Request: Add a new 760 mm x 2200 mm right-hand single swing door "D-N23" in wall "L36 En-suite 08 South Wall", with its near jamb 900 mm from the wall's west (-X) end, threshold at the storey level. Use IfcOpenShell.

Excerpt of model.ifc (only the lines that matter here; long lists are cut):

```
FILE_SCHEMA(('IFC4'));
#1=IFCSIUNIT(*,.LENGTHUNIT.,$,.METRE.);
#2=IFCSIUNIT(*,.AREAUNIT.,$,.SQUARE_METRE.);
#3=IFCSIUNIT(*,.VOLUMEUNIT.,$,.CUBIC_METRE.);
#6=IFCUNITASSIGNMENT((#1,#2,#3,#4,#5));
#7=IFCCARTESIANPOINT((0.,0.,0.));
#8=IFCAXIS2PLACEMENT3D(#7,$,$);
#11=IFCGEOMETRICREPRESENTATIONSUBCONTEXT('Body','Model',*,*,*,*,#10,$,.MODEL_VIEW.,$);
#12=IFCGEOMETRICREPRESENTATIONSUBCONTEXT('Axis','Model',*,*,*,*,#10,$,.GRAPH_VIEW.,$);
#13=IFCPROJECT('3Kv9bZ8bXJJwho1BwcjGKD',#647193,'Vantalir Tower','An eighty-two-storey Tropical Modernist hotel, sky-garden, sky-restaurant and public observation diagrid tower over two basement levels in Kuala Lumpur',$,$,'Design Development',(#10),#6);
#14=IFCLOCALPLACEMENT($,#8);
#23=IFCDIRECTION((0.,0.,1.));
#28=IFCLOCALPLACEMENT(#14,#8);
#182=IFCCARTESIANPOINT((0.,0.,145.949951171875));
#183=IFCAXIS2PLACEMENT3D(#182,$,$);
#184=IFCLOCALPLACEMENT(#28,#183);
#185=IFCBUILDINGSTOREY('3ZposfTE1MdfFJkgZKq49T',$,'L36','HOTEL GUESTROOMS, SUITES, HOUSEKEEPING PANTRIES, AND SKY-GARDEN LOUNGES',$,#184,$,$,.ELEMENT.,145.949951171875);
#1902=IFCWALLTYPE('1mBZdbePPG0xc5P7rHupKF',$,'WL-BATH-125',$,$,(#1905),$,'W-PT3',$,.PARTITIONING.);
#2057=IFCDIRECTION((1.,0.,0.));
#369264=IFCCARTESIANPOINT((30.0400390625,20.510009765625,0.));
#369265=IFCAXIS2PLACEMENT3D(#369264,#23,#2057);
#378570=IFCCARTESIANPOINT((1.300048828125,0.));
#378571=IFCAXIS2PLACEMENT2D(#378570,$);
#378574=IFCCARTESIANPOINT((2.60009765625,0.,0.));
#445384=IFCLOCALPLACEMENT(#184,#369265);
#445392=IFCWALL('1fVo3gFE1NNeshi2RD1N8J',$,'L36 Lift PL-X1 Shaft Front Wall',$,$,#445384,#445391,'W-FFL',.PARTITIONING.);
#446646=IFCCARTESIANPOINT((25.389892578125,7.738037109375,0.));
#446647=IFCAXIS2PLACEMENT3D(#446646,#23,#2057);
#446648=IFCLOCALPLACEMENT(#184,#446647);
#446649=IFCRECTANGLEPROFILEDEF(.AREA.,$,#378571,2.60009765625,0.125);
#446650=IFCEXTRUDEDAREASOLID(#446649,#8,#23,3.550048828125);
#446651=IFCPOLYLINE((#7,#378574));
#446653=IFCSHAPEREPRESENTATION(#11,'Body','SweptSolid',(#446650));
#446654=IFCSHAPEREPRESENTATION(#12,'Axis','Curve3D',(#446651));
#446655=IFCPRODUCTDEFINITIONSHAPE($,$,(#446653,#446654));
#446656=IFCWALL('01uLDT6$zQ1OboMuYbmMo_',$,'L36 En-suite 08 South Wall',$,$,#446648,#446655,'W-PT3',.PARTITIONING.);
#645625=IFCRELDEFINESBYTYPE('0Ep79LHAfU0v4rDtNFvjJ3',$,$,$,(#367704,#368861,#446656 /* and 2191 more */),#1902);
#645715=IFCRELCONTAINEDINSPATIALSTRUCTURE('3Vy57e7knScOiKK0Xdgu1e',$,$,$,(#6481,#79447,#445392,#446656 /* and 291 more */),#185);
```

```python
import numpy as np
import ifcopenshell
import ifcopenshell.api.feature
import ifcopenshell.api.geometry
import ifcopenshell.api.root
import ifcopenshell.api.spatial
import ifcopenshell.geom
import ifcopenshell.util.element
import ifcopenshell.util.placement
import ifcopenshell.util.representation
import ifcopenshell.util.shape
import ifcopenshell.util.unit

model = ifcopenshell.open("model.ifc")
unit_scale = ifcopenshell.util.unit.calculate_unit_scale(model)
settings = ifcopenshell.geom.settings()


def volume(element):
    """Net volume in cubic metres, openings subtracted."""
    shape = ifcopenshell.geom.create_shape(settings, element)
    return ifcopenshell.util.shape.get_volume(shape.geometry)


wall = model.by_guid("01uLDT6$zQ1OboMuYbmMo_")
storey = ifcopenshell.util.element.get_container(wall, ifc_class="IfcBuildingStorey")
context = ifcopenshell.util.representation.get_context(model, "Model", "Body", "MODEL_VIEW")
before = volume(wall)

width, height, from_end, sill = 0.76, 2.2, 0.9, 0.0  # metres

# The wall runs along its own X axis, and the end named is its -X end.
wall_shape = ifcopenshell.geom.create_shape(settings, wall)
x, y, z = ifcopenshell.util.shape.get_vertices(wall_shape.geometry).T
start = x.min() + from_end
face, thickness = float(y.min()), float(y.max() - y.min())
wall_matrix = ifcopenshell.util.placement.get_local_placement(wall.ObjectPlacement)
level = ifcopenshell.util.placement.get_local_placement(storey.ObjectPlacement)[2, 3]


def in_wall(x, y):
    """Placement at x, y metres in the wall's axes, at sill height."""
    matrix = wall_matrix.copy()
    matrix[:, 3] = wall_matrix @ np.array([x / unit_scale, y / unit_scale, 0.0, 1.0])
    matrix[2, 3] = level + sill / unit_scale
    return matrix


# Opening: a box that overshoots both wall faces by 50 mm.
opening = ifcopenshell.api.root.create_entity(model, ifc_class="IfcOpeningElement", predefined_type="OPENING")
box = ifcopenshell.api.geometry.add_wall_representation(
    model, context=context, length=width, height=height, thickness=thickness + 0.1
)
ifcopenshell.api.geometry.assign_representation(model, product=opening, representation=box)
ifcopenshell.api.geometry.edit_object_placement(model, product=opening, matrix=in_wall(start, face - 0.05), is_si=False)
ifcopenshell.api.feature.add_feature(model, feature=opening, element=wall)

door = ifcopenshell.api.root.create_entity(model, ifc_class="IfcDoor", name="D-N23", predefined_type="DOOR")
door.OverallWidth, door.OverallHeight = width / unit_scale, height / unit_scale
door.OperationType = "SINGLE_SWING_RIGHT"
body = ifcopenshell.api.geometry.add_door_representation(
    model,
    context=context,
    overall_width=door.OverallWidth,
    overall_height=door.OverallHeight,
    operation_type="SINGLE_SWING_RIGHT",
    lining_properties={"LiningDepth": thickness / unit_scale, "ThresholdDepth": thickness / unit_scale},
)
ifcopenshell.api.geometry.assign_representation(model, product=door, representation=body)
ifcopenshell.api.spatial.assign_container(model, products=[door], relating_structure=storey)
ifcopenshell.api.feature.add_filling(model, opening=opening, element=door)

# The lining spans the wall, so the door starts at the wall face.
ifcopenshell.api.geometry.edit_object_placement(model, product=door, matrix=in_wall(start, face), is_si=False)

after = volume(wall)

print(f"wall volume {before:.3f} -> {after:.3f} m3")

model.write("model-out.ifc")
```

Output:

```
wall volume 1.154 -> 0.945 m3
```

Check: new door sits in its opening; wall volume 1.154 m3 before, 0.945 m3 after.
